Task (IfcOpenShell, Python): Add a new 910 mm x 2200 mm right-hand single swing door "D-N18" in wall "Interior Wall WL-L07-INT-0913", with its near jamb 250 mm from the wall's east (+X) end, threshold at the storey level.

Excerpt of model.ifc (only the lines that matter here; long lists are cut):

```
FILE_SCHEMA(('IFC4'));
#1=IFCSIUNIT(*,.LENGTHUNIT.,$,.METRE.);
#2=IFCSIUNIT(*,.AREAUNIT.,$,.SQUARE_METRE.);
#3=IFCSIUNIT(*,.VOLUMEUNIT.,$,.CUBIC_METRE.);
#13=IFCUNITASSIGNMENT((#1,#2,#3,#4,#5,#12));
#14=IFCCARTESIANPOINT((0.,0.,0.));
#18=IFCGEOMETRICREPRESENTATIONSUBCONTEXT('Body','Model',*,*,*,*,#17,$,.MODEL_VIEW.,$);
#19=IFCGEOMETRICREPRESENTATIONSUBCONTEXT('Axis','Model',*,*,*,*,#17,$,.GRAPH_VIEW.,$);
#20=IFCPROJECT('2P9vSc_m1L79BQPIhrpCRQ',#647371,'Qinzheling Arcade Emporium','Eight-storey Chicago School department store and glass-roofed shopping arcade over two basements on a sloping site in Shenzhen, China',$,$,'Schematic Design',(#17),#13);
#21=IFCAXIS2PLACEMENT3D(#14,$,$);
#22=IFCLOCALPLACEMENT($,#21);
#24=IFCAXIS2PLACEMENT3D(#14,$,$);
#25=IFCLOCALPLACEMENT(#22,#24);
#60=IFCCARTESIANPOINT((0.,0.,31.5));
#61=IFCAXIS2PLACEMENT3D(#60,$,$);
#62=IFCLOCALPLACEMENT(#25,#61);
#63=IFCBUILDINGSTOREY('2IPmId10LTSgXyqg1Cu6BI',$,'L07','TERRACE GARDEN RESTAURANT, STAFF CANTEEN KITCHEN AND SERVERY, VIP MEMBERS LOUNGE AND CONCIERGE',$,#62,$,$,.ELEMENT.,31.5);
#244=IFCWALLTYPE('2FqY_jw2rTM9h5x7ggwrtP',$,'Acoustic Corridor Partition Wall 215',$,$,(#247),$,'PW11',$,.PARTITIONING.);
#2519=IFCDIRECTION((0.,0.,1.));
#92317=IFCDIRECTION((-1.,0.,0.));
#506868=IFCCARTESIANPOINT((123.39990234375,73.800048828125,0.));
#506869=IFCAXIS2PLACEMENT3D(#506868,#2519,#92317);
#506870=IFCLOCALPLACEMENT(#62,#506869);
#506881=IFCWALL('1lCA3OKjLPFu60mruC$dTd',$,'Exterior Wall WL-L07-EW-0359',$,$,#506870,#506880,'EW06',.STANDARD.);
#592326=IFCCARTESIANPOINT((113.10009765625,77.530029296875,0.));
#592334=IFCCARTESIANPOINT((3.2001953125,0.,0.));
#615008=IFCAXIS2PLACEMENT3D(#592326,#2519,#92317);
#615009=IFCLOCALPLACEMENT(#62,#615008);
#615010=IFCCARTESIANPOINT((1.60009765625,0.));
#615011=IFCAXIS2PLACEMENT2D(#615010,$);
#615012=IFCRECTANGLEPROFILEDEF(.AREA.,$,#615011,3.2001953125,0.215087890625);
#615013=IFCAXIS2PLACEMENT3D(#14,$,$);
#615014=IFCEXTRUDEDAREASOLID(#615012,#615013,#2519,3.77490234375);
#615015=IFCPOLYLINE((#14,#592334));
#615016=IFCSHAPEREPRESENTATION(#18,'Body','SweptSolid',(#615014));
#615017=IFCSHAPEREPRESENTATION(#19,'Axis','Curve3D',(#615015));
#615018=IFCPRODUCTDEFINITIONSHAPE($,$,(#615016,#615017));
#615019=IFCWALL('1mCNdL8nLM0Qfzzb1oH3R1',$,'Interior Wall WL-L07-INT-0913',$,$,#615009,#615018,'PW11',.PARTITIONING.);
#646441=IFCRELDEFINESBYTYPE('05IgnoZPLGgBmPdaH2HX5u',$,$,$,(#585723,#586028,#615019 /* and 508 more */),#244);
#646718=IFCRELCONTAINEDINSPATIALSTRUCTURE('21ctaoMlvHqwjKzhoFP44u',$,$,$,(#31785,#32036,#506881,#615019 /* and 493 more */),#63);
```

```python
import numpy as np
import ifcopenshell
import ifcopenshell.api.feature
import ifcopenshell.api.geometry
import ifcopenshell.api.root
import ifcopenshell.api.spatial
import ifcopenshell.geom
import ifcopenshell.util.element
import ifcopenshell.util.placement
import ifcopenshell.util.representation
import ifcopenshell.util.shape
import ifcopenshell.util.unit

model = ifcopenshell.open("model.ifc")
unit_scale = ifcopenshell.util.unit.calculate_unit_scale(model)
settings = ifcopenshell.geom.settings()


def volume(element):
    """Net volume in cubic metres, openings subtracted."""
    shape = ifcopenshell.geom.create_shape(settings, element)
    return ifcopenshell.util.shape.get_volume(shape.geometry)


wall = model.by_id(615019)
storey = ifcopenshell.util.element.get_container(wall, ifc_class="IfcBuildingStorey")
context = ifcopenshell.util.representation.get_context(model, "Model", "Body", "MODEL_VIEW")
before = volume(wall)

width, height, from_end, sill = 0.91, 2.2, 0.25, 0.0  # metres

# The wall runs along its own X axis, and the end named is its -X end.
wall_shape = ifcopenshell.geom.create_shape(settings, wall)
x, y, z = ifcopenshell.util.shape.get_vertices(wall_shape.geometry).T
start = x.min() + from_end
face, thickness = float(y.min()), float(y.max() - y.min())
wall_matrix = ifcopenshell.util.placement.get_local_placement(wall.ObjectPlacement)
level = ifcopenshell.util.placement.get_local_placement(storey.ObjectPlacement)[2, 3]


def in_wall(x, y):
    """Placement at x, y metres in the wall's axes, at sill height."""
    matrix = wall_matrix.copy()
    matrix[:, 3] = wall_matrix @ np.array([x / unit_scale, y / unit_scale, 0.0, 1.0])
    matrix[2, 3] = level + sill / unit_scale
    return matrix


# Opening: a box that overshoots both wall faces by 50 mm.
opening = ifcopenshell.api.root.create_entity(model, ifc_class="IfcOpeningElement", predefined_type="OPENING")
box = ifcopenshell.api.geometry.add_wall_representation(
    model, context=context, length=width, height=height, thickness=thickness + 0.1
)
ifcopenshell.api.geometry.assign_representation(model, product=opening, representation=box)
ifcopenshell.api.geometry.edit_object_placement(model, product=opening, matrix=in_wall(start, face - 0.05), is_si=False)
ifcopenshell.api.feature.add_feature(model, feature=opening, element=wall)

door = ifcopenshell.api.root.create_entity(model, ifc_class="IfcDoor", name="D-N18", predefined_type="DOOR")
door.OverallWidth, door.OverallHeight = width / unit_scale, height / unit_scale
door.OperationType = "SINGLE_SWING_RIGHT"
body = ifcopenshell.api.geometry.add_door_representation(
    model,
    context=context,
    overall_width=door.OverallWidth,
    overall_height=door.OverallHeight,
    operation_type="SINGLE_SWING_RIGHT",
    lining_properties={"LiningDepth": thickness / unit_scale, "ThresholdDepth": thickness / unit_scale},
)
ifcopenshell.api.geometry.assign_representation(model, product=door, representation=body)
ifcopenshell.api.spatial.assign_container(model, products=[door], relating_structure=storey)
ifcopenshell.api.feature.add_filling(model, opening=opening, element=door)

# The lining spans the wall, so the door starts at the wall face.
ifcopenshell.api.geometry.edit_object_placement(model, product=door, matrix=in_wall(start, face), is_si=False)

after = volume(wall)

print(f"wall volume {before:.3f} -> {after:.3f} m3")

model.write("model_updated.ifc")
```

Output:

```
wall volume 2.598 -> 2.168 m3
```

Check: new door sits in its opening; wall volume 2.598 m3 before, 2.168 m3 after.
